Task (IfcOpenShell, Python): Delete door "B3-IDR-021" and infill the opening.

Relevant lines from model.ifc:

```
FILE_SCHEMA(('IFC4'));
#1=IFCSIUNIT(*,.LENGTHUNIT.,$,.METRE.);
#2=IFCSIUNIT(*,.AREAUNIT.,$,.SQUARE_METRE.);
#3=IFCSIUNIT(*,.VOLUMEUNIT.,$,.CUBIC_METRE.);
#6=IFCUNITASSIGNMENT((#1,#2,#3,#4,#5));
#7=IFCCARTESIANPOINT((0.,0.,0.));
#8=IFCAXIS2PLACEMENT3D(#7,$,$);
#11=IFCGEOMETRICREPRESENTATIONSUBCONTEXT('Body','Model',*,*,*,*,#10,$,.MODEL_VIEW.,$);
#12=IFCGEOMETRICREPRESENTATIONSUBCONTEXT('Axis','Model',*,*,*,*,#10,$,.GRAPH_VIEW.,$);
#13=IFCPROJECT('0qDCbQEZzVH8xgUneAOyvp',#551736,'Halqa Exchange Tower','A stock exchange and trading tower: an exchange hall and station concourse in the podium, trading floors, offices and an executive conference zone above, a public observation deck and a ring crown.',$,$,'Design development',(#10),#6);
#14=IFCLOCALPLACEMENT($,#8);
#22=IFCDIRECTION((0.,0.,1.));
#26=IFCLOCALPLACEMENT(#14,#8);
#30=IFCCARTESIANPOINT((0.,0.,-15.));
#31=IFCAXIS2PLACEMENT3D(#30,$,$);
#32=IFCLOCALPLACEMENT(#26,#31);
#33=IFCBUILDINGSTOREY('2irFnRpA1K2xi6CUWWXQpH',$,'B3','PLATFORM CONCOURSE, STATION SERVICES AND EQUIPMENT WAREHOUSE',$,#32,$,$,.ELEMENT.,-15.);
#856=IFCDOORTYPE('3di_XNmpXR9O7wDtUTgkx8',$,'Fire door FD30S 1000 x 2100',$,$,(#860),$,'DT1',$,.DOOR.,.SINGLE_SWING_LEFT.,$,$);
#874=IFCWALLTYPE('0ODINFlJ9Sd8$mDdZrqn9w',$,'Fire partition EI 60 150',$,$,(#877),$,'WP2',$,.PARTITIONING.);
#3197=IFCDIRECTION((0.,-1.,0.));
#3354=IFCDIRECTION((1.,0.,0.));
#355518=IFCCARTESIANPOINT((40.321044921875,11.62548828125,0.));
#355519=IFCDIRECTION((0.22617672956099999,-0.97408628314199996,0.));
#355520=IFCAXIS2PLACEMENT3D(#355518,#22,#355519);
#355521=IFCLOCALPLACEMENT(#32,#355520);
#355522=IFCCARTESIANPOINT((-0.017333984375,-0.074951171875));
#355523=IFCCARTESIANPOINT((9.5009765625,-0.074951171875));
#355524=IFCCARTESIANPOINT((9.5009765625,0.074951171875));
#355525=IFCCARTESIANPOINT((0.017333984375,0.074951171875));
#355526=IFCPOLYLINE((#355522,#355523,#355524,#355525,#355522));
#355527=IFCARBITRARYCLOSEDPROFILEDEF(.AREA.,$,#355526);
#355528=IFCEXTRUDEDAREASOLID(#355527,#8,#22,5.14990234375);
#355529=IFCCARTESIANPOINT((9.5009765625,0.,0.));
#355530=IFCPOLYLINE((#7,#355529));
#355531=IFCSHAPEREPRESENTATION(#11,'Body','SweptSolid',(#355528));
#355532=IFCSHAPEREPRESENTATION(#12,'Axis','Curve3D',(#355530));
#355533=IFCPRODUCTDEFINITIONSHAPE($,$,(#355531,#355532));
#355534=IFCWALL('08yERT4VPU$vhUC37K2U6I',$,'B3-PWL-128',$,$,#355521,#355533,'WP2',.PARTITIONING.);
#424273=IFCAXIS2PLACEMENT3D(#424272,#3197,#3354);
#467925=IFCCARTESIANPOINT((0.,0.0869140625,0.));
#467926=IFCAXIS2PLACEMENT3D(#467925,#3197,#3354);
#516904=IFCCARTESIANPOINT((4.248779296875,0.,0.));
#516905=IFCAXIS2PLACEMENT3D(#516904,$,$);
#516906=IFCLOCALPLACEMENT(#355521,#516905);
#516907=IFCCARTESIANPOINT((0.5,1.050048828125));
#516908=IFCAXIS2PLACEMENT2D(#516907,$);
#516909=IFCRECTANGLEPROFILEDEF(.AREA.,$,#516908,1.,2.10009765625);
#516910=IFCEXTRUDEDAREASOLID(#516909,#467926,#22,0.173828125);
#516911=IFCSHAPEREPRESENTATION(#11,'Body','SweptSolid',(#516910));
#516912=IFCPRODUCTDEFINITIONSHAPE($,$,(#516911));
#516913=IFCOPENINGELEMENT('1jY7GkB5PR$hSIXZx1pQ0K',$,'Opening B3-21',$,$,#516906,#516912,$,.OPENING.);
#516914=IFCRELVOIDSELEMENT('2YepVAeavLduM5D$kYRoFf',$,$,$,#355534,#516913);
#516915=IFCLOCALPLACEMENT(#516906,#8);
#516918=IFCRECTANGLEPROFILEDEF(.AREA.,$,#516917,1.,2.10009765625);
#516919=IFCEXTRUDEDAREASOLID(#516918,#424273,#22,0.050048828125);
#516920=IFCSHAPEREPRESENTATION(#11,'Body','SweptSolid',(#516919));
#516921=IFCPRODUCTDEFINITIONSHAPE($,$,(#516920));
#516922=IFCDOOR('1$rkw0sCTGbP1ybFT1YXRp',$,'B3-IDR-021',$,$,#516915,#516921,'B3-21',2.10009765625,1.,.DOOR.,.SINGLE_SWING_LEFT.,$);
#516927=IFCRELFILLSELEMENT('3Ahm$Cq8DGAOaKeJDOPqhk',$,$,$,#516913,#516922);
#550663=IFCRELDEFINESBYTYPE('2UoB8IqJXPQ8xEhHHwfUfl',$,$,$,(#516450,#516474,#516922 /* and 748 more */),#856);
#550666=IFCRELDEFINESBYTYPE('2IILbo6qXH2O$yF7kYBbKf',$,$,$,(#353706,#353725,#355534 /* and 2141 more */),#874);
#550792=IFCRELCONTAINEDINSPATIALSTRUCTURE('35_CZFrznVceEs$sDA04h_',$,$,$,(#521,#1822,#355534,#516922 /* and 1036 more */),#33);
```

```python
import ifcopenshell
import ifcopenshell.api.feature
import ifcopenshell.api.root
import ifcopenshell.geom
import ifcopenshell.util.shape

model = ifcopenshell.open("model.ifc")
settings = ifcopenshell.geom.settings()


def volume(element):
    """Net volume in cubic metres, openings subtracted."""
    shape = ifcopenshell.geom.create_shape(settings, element)
    return ifcopenshell.util.shape.get_volume(shape.geometry)


door = model.by_guid("1$rkw0sCTGbP1ybFT1YXRp")
opening = door.FillsVoids[0].RelatingOpeningElement
wall = opening.VoidsElements[0].RelatingBuildingElement
before = volume(wall)

ifcopenshell.api.root.remove_product(model, product=door)
ifcopenshell.api.feature.remove_feature(model, feature=opening)

after = volume(wall)

print(f"wall volume {before:.3f} -> {after:.3f} m3")

model.write("model_rev.ifc")
```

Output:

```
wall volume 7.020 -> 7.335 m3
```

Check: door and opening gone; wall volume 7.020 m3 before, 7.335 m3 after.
